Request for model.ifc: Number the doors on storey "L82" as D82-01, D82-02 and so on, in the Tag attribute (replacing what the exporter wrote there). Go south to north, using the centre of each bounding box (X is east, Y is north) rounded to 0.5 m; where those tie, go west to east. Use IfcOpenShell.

First a look at what the model holds.

```python
import ifcopenshell
import ifcopenshell.util.element
import ifcopenshell.util.placement

model = ifcopenshell.open("model.ifc")
print(model.schema)
storey = next(s for s in model.by_type("IfcBuildingStorey") if s.Name == "L82")
doors = [e for e in ifcopenshell.util.element.get_decomposition(storey) if e.is_a("IfcDoor")]
for e in sorted(doors, key=lambda e: e.id()):
    origin = ifcopenshell.util.placement.get_local_placement(e.ObjectPlacement)[:3, 3]
    print(e.id(), e.Tag, e.Name, origin.round(2) + 0.0, sep=" | ")
```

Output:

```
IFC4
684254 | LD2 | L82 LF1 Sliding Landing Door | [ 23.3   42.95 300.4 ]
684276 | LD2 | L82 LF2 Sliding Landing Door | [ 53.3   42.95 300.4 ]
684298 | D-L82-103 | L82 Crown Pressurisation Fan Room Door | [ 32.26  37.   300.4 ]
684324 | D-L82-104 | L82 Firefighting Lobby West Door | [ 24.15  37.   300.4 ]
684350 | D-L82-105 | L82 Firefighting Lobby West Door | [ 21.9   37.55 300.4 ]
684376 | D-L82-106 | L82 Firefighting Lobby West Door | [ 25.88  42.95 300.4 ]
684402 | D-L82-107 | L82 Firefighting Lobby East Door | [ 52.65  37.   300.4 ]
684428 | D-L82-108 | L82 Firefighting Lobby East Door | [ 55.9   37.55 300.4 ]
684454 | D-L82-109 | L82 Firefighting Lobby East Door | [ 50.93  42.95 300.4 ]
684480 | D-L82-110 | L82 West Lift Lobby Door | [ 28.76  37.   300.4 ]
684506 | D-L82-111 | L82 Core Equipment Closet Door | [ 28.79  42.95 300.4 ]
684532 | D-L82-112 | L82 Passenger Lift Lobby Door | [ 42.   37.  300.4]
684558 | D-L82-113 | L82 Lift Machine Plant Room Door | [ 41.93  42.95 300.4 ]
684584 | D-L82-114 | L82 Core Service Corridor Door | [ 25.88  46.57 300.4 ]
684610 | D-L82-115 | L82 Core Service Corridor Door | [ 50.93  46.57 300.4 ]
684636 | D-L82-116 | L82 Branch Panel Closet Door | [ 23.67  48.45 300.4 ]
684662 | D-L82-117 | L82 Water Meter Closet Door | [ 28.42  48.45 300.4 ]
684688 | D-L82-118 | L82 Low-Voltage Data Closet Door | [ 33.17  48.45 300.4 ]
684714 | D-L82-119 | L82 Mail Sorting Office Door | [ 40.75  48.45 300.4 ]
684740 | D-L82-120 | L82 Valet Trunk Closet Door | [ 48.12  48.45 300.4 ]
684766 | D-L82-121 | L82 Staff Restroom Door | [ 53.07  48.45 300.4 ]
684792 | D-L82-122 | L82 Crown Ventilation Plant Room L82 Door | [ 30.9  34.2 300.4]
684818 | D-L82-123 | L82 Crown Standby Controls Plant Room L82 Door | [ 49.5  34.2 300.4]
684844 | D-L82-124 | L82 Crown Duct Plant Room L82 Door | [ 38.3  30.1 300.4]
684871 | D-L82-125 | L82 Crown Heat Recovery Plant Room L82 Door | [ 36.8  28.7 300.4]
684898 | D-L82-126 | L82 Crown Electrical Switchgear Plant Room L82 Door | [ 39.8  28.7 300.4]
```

```python
import ifcopenshell
import ifcopenshell.geom
import ifcopenshell.util.element
import ifcopenshell.util.shape

model = ifcopenshell.open("model.ifc")
settings = ifcopenshell.geom.settings()
settings.set("use-world-coords", True)


def centre(element):
    shape = ifcopenshell.geom.create_shape(settings, element)
    return ifcopenshell.util.shape.get_bbox_centroid(shape.geometry)


storey = next(s for s in model.by_type("IfcBuildingStorey") if s.Name == "L82")
doors = [e for e in ifcopenshell.util.element.get_decomposition(storey) if e.is_a("IfcDoor")]

# Insertion points can sit at a corner or the storey origin, so sort by the geometry (in metres).
centres = {e: centre(e) for e in doors}
doors.sort(key=lambda e: (round(centres[e][1] / 0.5), centres[e][0]))

for i, e in enumerate(doors, start=1):
    number = f"D82-{i:02d}"
    e.Tag = number
    print(e.id(), number)

model.write("model_v2.ifc")
```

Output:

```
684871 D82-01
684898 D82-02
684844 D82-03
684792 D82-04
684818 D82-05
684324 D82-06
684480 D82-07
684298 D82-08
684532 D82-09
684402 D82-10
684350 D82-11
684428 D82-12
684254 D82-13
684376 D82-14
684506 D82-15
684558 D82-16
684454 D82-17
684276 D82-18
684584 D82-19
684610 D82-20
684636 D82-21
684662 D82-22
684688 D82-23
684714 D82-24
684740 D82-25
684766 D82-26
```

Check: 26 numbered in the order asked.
